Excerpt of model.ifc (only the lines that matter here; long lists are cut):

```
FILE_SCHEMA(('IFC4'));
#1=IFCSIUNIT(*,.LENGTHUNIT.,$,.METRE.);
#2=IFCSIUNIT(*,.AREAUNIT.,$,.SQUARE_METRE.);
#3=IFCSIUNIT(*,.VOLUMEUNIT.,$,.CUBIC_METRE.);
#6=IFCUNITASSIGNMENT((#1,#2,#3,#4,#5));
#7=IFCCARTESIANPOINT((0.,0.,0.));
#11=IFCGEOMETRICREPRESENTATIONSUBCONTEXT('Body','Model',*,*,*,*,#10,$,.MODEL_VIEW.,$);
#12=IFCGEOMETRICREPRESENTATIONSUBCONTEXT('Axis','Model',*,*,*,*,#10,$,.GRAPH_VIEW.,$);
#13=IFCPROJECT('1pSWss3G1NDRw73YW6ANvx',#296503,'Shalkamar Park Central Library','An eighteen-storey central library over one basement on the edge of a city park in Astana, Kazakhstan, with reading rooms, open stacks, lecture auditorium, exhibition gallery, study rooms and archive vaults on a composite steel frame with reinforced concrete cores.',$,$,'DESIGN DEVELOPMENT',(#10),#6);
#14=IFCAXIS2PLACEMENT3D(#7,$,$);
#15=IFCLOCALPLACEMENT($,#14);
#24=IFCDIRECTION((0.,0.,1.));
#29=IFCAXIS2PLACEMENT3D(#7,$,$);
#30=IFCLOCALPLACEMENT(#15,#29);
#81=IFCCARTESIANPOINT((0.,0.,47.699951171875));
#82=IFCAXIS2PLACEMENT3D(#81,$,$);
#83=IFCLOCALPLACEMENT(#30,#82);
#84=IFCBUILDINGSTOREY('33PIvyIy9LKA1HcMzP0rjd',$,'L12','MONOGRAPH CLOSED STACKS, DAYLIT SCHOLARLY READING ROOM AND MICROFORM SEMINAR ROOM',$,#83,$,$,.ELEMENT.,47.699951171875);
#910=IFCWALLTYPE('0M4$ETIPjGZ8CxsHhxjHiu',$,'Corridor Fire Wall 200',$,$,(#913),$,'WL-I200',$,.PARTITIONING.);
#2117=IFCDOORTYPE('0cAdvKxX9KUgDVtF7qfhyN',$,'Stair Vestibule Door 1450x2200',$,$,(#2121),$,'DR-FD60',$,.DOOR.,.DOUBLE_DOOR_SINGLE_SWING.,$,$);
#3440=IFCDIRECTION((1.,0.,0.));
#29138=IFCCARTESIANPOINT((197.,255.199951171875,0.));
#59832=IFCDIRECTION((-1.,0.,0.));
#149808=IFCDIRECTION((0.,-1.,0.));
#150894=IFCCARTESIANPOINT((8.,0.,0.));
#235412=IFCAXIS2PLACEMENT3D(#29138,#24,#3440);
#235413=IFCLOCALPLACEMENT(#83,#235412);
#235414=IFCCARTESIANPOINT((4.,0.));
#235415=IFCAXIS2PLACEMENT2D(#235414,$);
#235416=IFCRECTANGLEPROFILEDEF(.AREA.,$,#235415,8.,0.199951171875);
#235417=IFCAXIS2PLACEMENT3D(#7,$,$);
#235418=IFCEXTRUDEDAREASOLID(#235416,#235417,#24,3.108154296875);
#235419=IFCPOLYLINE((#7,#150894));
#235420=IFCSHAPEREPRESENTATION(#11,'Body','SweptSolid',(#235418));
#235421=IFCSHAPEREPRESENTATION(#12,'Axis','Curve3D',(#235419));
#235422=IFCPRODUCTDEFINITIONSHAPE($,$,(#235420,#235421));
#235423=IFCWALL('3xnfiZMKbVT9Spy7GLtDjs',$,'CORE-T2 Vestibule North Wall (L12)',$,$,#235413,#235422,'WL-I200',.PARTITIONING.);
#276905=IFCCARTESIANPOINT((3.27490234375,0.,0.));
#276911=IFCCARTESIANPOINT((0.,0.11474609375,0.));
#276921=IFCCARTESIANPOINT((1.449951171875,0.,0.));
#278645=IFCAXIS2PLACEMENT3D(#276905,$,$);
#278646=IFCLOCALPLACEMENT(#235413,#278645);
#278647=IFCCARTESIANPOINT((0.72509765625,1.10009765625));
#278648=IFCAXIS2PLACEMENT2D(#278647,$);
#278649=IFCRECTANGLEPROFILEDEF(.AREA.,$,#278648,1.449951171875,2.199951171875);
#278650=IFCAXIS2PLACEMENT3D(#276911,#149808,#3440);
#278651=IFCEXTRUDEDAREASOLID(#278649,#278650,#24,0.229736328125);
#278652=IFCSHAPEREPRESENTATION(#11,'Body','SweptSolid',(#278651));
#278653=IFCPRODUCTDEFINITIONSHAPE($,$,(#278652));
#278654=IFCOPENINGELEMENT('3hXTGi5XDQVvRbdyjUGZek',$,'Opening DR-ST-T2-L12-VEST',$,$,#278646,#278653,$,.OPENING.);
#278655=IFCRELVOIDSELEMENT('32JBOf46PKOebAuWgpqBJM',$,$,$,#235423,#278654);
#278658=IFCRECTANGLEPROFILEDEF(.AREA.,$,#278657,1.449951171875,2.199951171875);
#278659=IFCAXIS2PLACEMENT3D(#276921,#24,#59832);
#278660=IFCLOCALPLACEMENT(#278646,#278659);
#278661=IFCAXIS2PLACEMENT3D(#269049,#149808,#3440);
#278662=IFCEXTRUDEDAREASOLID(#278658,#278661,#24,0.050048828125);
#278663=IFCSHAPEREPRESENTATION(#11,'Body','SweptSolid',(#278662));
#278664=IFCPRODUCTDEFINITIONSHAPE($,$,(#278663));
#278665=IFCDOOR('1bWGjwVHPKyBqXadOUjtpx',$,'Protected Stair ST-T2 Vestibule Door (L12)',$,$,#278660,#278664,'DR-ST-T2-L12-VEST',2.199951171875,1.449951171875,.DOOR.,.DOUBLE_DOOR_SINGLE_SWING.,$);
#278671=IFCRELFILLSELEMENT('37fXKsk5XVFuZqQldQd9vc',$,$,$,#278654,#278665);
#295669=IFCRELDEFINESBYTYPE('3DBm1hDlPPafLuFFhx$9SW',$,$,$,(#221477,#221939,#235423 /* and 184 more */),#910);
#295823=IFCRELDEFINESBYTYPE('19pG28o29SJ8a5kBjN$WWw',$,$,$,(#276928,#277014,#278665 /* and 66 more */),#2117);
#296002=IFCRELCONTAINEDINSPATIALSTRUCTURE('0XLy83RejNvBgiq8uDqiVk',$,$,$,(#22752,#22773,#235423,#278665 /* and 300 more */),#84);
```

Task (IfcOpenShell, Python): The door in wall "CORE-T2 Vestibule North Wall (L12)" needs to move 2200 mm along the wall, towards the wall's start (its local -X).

```python
import ifcopenshell
import ifcopenshell.api.geometry
import ifcopenshell.util.placement
import ifcopenshell.util.unit

model = ifcopenshell.open("model.ifc")
unit_scale = ifcopenshell.util.unit.calculate_unit_scale(model)

door = model.by_guid("1bWGjwVHPKyBqXadOUjtpx")
opening = door.FillsVoids[0].RelatingOpeningElement
wall = opening.VoidsElements[0].RelatingBuildingElement

wall_matrix = ifcopenshell.util.placement.get_local_placement(wall.ObjectPlacement)
shift = wall_matrix[:3, 0] * -2.2 / unit_scale
before = ifcopenshell.util.placement.get_local_placement(door.ObjectPlacement)[:3, 3].copy()

# The door is placed relative to its opening, so it follows when the opening moves.
matrix = ifcopenshell.util.placement.get_local_placement(opening.ObjectPlacement)
matrix[:3, 3] += shift
ifcopenshell.api.geometry.edit_object_placement(
    model, product=opening, matrix=matrix, is_si=False, should_transform_children=True
)

after = ifcopenshell.util.placement.get_local_placement(door.ObjectPlacement)[:3, 3]
print("door moved by", (after - before).round(3) + 0.0)

model.write("model_updated.ifc")
```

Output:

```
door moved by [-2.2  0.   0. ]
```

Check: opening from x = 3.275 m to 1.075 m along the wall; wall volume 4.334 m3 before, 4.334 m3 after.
